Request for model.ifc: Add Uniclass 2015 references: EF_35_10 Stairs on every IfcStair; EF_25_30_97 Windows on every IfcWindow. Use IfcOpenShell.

First a look at what the model holds.

```python
import ifcopenshell

model = ifcopenshell.open("model.ifc")
print(model.schema)
print("classifications:", [c.Name for c in model.by_type("IfcClassification")])
for ifc_class in ("IfcDoor", "IfcRoof", "IfcStair", "IfcWall", "IfcWindow"):
    print(ifc_class, len(model.by_type(ifc_class)))
```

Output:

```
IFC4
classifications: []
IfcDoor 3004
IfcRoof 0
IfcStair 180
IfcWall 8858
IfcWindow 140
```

```python
import ifcopenshell
import ifcopenshell.api.classification

model = ifcopenshell.open("model.ifc")

system = ifcopenshell.api.classification.add_classification(model, classification="Uniclass 2015")

codes = {
    "IfcStair": ("EF_35_10", "Stairs"),
    "IfcWindow": ("EF_25_30_97", "Windows"),
}
for ifc_class, (code, name) in codes.items():
    products = model.by_type(ifc_class)
    ifcopenshell.api.classification.add_reference(
        model, products=products, classification=system, identification=code, name=name
    )
    print(code, len(products))

model.write("model_edited.ifc")
```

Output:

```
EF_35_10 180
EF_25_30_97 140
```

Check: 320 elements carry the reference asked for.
